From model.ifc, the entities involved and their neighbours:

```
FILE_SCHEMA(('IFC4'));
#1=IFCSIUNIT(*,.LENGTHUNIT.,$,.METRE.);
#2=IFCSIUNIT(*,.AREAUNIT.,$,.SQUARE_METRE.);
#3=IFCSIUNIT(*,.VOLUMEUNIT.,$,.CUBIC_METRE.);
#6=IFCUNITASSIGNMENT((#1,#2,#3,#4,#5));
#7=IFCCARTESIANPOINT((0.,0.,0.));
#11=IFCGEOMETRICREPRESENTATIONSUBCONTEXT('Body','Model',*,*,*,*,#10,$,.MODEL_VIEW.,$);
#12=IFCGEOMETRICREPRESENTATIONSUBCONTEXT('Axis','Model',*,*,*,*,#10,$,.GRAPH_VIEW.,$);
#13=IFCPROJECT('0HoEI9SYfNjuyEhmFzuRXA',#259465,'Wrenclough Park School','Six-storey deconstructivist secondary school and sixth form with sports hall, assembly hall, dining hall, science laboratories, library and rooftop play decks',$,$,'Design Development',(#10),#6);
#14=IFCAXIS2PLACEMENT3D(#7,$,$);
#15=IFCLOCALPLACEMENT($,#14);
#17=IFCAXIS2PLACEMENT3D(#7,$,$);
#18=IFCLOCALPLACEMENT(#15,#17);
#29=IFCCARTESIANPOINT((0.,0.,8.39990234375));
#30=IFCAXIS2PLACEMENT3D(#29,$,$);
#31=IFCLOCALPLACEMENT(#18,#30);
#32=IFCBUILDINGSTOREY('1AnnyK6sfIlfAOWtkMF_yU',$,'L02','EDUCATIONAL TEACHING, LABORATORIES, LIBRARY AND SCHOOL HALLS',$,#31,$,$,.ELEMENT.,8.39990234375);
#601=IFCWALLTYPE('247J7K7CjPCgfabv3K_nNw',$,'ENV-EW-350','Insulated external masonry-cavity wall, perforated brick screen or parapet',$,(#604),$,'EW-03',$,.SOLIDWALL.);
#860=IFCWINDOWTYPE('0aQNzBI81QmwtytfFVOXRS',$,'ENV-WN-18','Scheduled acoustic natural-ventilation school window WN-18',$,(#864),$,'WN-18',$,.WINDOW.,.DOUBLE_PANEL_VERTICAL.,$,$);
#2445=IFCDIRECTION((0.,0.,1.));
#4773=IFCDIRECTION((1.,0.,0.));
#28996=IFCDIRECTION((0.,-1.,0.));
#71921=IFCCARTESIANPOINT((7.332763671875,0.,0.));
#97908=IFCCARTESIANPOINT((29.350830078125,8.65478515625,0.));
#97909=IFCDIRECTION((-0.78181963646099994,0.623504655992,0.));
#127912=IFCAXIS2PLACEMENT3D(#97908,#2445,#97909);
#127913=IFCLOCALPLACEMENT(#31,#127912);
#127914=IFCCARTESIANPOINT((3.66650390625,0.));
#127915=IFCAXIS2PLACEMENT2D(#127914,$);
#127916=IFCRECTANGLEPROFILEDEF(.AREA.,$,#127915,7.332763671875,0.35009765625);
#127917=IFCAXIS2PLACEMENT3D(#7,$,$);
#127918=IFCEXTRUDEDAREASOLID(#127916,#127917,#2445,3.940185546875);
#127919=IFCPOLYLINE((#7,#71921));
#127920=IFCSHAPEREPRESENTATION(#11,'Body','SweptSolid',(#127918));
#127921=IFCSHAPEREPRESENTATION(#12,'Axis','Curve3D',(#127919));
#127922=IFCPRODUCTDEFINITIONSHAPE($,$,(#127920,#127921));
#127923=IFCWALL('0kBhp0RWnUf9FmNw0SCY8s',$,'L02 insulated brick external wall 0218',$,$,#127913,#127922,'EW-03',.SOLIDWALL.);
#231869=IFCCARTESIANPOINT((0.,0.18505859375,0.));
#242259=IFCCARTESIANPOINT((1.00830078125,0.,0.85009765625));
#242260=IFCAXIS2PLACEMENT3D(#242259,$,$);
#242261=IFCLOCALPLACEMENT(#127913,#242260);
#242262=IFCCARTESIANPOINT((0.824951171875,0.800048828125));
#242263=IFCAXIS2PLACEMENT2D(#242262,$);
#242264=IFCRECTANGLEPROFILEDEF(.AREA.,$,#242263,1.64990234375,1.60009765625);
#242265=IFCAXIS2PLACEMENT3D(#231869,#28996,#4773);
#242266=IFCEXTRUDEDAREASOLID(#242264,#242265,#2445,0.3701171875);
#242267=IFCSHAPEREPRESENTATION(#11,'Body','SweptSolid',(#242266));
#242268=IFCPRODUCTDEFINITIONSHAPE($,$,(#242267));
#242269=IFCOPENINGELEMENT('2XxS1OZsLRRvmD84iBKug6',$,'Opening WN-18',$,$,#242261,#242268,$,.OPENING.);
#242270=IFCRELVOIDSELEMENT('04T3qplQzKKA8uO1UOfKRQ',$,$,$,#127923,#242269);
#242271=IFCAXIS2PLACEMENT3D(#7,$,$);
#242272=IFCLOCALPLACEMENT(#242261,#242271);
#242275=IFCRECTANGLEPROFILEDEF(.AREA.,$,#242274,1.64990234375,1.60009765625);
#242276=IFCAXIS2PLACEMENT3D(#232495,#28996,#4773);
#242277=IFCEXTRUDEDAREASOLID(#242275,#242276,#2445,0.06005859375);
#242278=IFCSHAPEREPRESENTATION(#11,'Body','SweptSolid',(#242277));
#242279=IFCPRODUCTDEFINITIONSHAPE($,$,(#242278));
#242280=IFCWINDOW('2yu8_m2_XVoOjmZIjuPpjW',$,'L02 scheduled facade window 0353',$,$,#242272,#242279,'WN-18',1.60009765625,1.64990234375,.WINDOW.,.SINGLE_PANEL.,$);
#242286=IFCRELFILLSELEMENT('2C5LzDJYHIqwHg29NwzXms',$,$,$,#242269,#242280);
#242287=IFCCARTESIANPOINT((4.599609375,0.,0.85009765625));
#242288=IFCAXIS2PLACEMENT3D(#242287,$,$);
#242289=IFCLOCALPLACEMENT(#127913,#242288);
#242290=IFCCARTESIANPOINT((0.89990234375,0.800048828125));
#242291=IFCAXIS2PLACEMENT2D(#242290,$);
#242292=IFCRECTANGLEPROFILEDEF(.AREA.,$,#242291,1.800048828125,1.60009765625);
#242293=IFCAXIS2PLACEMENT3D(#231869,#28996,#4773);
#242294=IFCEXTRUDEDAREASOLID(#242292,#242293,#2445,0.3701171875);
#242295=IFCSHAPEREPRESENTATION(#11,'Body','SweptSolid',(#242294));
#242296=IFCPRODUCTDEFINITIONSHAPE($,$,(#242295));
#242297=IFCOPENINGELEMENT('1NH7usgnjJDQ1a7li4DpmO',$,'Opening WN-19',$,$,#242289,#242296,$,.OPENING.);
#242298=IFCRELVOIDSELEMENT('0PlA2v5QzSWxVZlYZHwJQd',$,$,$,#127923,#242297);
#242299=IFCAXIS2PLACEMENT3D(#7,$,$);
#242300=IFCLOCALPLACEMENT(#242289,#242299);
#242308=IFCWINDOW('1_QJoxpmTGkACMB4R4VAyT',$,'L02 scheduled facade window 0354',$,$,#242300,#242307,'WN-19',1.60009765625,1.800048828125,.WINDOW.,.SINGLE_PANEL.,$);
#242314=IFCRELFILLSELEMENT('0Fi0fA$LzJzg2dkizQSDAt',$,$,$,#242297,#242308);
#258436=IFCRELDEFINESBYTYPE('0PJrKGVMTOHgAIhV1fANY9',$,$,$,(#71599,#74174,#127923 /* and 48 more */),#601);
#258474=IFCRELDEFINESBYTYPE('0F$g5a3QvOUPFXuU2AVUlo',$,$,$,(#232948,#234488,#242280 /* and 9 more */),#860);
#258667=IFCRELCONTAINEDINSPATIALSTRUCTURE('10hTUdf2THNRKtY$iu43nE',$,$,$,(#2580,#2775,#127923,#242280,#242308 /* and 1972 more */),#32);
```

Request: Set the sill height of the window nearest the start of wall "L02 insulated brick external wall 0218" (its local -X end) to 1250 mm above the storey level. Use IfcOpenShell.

```python
import numpy as np
import ifcopenshell
import ifcopenshell.api.geometry
import ifcopenshell.geom
import ifcopenshell.util.element
import ifcopenshell.util.placement
import ifcopenshell.util.shape
import ifcopenshell.util.unit

model = ifcopenshell.open("model.ifc")
unit_scale = ifcopenshell.util.unit.calculate_unit_scale(model)

window = model.by_guid("2yu8_m2_XVoOjmZIjuPpjW")
opening = window.FillsVoids[0].RelatingOpeningElement
storey = ifcopenshell.util.element.get_container(window, ifc_class="IfcBuildingStorey")
level = ifcopenshell.util.placement.get_local_placement(storey.ObjectPlacement)[2, 3]

# The opening's origin need not be at the sill, so measure its lowest point.
shape = ifcopenshell.geom.create_shape(ifcopenshell.geom.settings(), opening)
bottom = ifcopenshell.util.shape.get_shape_bottom_elevation(shape, shape.geometry) / unit_scale
dz = level + 1.25 / unit_scale - bottom

shift = np.array([0.0, 0.0, dz])
# The window is placed relative to its opening, so it follows when the opening moves.
matrix = ifcopenshell.util.placement.get_local_placement(opening.ObjectPlacement)
matrix[:3, 3] += shift
ifcopenshell.api.geometry.edit_object_placement(
    model, product=opening, matrix=matrix, is_si=False, should_transform_children=True
)

print(f"moved by {dz * unit_scale:+.3f} m")

model.write("model_edited.ifc")
```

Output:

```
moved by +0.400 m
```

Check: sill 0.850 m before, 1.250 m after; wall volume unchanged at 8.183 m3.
